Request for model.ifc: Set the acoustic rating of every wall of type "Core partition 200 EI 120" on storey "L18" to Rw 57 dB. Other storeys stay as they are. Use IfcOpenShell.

First a look at what the model holds.

```python
import ifcopenshell
import ifcopenshell.util.element

model = ifcopenshell.open("model.ifc")
print(model.schema)
storey = next(s for s in model.by_type("IfcBuildingStorey") if s.Name == "L18")
walls = [e for e in ifcopenshell.util.element.get_decomposition(storey) if e.is_a("IfcWall")]
seen = {}
for e in walls:
    element_type = ifcopenshell.util.element.get_type(e)
    key = (element_type.Name if element_type != e and element_type else None, ifcopenshell.util.element.get_pset(e, "Pset_WallCommon", "AcousticRating"))
    seen[key] = seen.get(key, 0) + 1
for (name, value), count in sorted(seen.items(), key=str):
    print(count, "x", name, "|", value)
```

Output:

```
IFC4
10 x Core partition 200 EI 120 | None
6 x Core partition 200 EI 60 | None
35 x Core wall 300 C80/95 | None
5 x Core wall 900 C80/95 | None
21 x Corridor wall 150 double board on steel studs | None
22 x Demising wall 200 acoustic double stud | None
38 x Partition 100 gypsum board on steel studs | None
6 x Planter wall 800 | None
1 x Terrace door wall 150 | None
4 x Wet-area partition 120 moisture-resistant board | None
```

```python
import ifcopenshell
import ifcopenshell.api.pset
import ifcopenshell.util.element

model = ifcopenshell.open("model.ifc")

storey = next(s for s in model.by_type("IfcBuildingStorey") if s.Name == "L18")
walls = [e for e in ifcopenshell.util.element.get_decomposition(storey) if e.is_a("IfcWall")]

count = 0
for e in walls:
    element_type = ifcopenshell.util.element.get_type(e)
    if element_type in (None, e) or element_type.Name != "Core partition 200 EI 120":
        continue
    found = ifcopenshell.util.element.get_pset(e, "Pset_WallCommon", should_inherit=False)
    if found:
        pset = model.by_id(found["id"])
        if len(ifcopenshell.util.element.get_elements_by_pset(pset)) > 1:
            pset = ifcopenshell.api.pset.unshare_pset(model, products=[e], pset=pset)[0]
    else:
        pset = ifcopenshell.api.pset.add_pset(model, product=e, name="Pset_WallCommon")
    ifcopenshell.api.pset.edit_pset(model, pset=pset, properties={"AcousticRating": "Rw 57 dB"})
    count += 1

print(count, "walls updated")

model.write("model_rev.ifc")
```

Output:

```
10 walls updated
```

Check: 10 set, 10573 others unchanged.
